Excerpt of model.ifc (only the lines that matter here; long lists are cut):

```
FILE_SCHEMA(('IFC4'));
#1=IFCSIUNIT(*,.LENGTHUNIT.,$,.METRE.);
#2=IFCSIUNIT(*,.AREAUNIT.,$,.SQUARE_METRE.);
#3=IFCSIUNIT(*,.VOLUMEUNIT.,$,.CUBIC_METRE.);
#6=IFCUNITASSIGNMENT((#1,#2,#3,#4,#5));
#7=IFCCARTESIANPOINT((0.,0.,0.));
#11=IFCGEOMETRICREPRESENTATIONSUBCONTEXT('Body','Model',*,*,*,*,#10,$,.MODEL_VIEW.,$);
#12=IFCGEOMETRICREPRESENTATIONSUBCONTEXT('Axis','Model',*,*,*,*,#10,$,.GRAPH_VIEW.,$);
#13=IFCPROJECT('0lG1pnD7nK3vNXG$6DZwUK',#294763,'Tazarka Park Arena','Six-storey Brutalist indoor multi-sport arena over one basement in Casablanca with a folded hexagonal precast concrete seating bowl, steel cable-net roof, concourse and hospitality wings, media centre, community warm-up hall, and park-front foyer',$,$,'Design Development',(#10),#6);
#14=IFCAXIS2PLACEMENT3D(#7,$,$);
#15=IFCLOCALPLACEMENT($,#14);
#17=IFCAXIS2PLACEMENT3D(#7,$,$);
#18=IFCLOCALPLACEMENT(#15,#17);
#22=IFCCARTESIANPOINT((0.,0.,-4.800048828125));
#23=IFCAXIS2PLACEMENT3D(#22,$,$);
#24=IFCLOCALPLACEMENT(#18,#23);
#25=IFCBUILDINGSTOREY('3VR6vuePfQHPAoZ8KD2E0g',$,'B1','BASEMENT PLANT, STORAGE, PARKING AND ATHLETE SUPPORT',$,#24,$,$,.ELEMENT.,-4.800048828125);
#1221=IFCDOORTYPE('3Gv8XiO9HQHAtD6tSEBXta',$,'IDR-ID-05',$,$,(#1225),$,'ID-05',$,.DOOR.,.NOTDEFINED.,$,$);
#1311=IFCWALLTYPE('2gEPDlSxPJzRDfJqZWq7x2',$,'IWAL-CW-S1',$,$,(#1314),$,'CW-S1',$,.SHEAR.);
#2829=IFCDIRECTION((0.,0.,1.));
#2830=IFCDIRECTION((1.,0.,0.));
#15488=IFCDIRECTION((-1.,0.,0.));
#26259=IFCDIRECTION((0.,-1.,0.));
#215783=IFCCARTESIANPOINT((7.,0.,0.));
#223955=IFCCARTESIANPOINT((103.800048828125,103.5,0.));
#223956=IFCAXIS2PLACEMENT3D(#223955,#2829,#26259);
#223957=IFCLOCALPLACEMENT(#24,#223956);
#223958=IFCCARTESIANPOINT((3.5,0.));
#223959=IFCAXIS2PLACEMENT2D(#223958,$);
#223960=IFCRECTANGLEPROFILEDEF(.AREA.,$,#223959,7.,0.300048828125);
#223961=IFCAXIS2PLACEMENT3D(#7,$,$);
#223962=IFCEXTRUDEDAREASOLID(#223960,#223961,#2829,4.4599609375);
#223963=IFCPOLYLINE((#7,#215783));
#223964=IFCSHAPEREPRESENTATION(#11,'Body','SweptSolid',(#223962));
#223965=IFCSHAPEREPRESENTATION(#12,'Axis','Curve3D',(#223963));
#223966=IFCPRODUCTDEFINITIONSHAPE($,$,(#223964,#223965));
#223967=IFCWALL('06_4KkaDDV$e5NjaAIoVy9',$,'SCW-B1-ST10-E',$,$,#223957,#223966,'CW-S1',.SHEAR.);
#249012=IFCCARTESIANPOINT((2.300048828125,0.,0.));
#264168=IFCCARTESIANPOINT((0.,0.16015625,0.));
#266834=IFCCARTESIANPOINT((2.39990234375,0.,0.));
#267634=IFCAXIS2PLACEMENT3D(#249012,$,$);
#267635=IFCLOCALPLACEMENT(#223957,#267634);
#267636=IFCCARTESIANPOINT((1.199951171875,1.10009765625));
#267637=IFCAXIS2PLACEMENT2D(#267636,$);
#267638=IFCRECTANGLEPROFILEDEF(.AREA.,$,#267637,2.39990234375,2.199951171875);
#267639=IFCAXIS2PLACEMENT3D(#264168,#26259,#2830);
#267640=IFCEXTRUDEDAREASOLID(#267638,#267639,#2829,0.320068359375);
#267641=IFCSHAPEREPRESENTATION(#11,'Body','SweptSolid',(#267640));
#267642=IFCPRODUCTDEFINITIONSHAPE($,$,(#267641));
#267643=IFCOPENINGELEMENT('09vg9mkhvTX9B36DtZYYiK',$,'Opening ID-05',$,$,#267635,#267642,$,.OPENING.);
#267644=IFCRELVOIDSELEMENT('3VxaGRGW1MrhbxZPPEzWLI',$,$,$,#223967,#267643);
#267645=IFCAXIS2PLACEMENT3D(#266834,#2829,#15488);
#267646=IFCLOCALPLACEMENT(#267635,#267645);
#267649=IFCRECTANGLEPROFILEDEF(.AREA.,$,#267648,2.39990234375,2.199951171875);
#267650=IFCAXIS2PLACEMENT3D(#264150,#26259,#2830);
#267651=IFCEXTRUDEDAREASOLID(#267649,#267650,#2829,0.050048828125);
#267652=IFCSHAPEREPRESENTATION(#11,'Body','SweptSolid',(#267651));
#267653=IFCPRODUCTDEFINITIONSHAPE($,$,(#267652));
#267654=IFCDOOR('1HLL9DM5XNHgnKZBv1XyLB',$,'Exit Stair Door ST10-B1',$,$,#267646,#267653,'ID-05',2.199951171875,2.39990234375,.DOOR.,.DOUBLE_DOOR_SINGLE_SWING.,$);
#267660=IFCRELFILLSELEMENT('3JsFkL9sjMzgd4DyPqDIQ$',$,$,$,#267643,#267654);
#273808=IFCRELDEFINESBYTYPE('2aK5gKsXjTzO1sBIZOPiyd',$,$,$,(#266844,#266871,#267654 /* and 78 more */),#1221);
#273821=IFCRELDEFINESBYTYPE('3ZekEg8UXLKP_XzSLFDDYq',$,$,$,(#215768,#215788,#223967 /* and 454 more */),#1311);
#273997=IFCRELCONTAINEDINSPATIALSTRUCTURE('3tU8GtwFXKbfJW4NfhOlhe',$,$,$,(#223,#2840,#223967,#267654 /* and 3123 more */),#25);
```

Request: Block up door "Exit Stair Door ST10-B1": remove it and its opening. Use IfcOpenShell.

```python
import ifcopenshell
import ifcopenshell.api.feature
import ifcopenshell.api.root
import ifcopenshell.geom
import ifcopenshell.util.shape

model = ifcopenshell.open("model.ifc")
settings = ifcopenshell.geom.settings()


def volume(element):
    """Net volume in cubic metres, openings subtracted."""
    shape = ifcopenshell.geom.create_shape(settings, element)
    return ifcopenshell.util.shape.get_volume(shape.geometry)


door = model.by_guid("1HLL9DM5XNHgnKZBv1XyLB")
opening = door.FillsVoids[0].RelatingOpeningElement
wall = opening.VoidsElements[0].RelatingBuildingElement
before = volume(wall)

ifcopenshell.api.root.remove_product(model, product=door)
ifcopenshell.api.feature.remove_feature(model, feature=opening)

after = volume(wall)

print(f"wall volume {before:.3f} -> {after:.3f} m3")

model.write("model_rev.ifc")
```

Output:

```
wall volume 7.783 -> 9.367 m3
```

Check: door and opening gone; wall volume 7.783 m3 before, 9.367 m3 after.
